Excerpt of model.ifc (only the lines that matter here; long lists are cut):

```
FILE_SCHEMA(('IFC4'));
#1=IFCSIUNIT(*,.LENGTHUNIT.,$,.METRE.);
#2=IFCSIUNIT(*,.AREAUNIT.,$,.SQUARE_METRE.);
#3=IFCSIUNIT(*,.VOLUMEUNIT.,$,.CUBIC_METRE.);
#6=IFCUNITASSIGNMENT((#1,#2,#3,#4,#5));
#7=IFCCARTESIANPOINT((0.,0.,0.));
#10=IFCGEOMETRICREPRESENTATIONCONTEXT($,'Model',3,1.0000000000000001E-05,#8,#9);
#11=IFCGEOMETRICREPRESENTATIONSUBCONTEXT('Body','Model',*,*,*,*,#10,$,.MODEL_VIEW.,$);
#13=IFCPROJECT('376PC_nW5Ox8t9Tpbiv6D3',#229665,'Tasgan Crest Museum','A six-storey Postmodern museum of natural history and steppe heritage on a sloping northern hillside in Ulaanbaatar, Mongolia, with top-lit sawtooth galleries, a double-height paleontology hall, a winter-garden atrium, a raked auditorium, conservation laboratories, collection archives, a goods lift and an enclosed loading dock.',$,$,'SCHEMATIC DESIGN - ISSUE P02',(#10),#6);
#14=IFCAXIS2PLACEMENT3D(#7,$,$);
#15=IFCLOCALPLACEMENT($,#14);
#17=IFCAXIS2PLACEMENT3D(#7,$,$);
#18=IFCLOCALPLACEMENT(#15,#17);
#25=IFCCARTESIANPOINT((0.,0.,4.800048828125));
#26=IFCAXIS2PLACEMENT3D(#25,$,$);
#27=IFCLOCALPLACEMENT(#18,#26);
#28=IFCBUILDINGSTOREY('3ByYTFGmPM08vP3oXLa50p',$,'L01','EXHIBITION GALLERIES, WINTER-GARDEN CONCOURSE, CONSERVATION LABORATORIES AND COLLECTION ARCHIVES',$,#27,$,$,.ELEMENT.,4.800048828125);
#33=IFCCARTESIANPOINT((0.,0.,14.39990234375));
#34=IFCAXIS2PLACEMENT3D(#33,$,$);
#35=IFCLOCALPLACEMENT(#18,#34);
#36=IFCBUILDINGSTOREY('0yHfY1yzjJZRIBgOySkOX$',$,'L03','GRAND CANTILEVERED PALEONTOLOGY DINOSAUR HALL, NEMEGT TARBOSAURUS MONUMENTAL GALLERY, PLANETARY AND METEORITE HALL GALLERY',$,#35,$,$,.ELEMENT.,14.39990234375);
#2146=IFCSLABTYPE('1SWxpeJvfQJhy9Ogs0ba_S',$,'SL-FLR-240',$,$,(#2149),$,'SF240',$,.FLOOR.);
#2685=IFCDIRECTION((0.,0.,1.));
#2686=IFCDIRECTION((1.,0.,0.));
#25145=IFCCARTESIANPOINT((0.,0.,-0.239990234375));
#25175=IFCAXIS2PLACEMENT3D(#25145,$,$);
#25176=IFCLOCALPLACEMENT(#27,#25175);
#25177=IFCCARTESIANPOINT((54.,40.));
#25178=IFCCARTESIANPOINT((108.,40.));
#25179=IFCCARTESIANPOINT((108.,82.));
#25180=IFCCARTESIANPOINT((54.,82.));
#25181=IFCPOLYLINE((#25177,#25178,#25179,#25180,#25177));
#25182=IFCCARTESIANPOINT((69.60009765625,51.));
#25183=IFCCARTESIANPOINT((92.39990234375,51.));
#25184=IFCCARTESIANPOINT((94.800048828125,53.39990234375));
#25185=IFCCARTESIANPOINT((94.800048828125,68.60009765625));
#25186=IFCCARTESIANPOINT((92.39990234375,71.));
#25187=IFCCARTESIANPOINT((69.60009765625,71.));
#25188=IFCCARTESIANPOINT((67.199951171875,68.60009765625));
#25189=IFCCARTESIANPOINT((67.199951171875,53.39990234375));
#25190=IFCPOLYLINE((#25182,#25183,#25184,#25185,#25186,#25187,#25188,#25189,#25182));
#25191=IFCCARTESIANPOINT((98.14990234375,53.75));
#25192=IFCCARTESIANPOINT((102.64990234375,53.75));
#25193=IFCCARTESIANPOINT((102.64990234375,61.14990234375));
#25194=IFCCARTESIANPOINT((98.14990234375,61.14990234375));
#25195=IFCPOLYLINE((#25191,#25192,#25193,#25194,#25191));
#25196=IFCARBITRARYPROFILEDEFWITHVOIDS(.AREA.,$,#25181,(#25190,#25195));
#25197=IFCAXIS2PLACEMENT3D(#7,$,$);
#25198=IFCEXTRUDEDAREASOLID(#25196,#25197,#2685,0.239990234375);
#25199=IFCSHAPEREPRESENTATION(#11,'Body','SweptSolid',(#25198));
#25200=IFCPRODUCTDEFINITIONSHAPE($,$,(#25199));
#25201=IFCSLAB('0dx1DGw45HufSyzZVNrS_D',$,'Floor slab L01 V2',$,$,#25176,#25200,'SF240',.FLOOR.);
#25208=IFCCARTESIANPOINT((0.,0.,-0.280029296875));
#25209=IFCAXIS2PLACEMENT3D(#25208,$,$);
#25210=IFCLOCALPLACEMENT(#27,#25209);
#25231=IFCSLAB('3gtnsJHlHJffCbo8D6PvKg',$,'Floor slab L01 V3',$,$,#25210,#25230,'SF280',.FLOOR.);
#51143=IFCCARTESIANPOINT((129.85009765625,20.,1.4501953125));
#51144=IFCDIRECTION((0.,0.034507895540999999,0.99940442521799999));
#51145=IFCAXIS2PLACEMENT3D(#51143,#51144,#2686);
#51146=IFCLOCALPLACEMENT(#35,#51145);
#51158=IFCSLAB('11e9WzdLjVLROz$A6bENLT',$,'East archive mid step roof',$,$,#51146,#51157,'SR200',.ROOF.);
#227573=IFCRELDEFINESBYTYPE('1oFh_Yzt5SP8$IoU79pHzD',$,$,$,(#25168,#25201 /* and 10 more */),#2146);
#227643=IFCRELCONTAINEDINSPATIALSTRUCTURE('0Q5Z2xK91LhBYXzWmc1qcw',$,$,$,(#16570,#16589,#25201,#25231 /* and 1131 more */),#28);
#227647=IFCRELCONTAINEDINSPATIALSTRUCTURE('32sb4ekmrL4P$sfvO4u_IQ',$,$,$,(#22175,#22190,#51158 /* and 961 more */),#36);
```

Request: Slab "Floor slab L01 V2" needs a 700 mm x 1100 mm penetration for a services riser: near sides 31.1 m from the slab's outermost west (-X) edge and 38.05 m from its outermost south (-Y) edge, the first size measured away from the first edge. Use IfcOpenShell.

```python
import numpy as np
import ifcopenshell
import ifcopenshell.api.feature
import ifcopenshell.api.geometry
import ifcopenshell.api.root
import ifcopenshell.geom
import ifcopenshell.util.placement
import ifcopenshell.util.representation
import ifcopenshell.util.shape
import ifcopenshell.util.unit

model = ifcopenshell.open("model.ifc")
unit_scale = ifcopenshell.util.unit.calculate_unit_scale(model)
settings = ifcopenshell.geom.settings()


def volume(element):
    """Net volume in cubic metres, openings subtracted."""
    shape = ifcopenshell.geom.create_shape(settings, element)
    return ifcopenshell.util.shape.get_volume(shape.geometry)


slab = model.by_guid("0dx1DGw45HufSyzZVNrS_D")
before = volume(slab)

# Extent in the slab's own axes, in metres. The edges named are its -X and -Y sides.
slab_shape = ifcopenshell.geom.create_shape(settings, slab)
vertices = ifcopenshell.util.shape.get_vertices(slab_shape.geometry)
x_min, y_min, bottom = vertices.min(axis=0)
top = vertices[:, 2].max()

opening = ifcopenshell.api.root.create_entity(model, ifc_class="IfcOpeningElement", name="Services riser opening", predefined_type="OPENING")
context = ifcopenshell.util.representation.get_context(model, "Model", "Body", "MODEL_VIEW")
width, depth = 0.7, 1.1
outline = [(0.0, 0.0), (width, 0.0), (width, depth), (0.0, depth), (0.0, 0.0)]
# Overshoot both faces by 50 mm so the cut is clean.
shape = ifcopenshell.api.geometry.add_slab_representation(
    model, context=context, depth=top - bottom + 0.1, polyline=outline
)
ifcopenshell.api.geometry.assign_representation(model, product=opening, representation=shape)

matrix = ifcopenshell.util.placement.get_local_placement(slab.ObjectPlacement)
matrix[:, 3] = matrix @ np.append(np.array([x_min + 31.1, y_min + 38.05, bottom - 0.05]) / unit_scale, 1.0)
ifcopenshell.api.geometry.edit_object_placement(model, product=opening, matrix=matrix, is_si=False)
ifcopenshell.api.feature.add_feature(model, feature=opening, element=slab)

after = volume(slab)

print(f"slab volume {before:.3f} -> {after:.3f} m3")

model.write("model_rev.ifc")
```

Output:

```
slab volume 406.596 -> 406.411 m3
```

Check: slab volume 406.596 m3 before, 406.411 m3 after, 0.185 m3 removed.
